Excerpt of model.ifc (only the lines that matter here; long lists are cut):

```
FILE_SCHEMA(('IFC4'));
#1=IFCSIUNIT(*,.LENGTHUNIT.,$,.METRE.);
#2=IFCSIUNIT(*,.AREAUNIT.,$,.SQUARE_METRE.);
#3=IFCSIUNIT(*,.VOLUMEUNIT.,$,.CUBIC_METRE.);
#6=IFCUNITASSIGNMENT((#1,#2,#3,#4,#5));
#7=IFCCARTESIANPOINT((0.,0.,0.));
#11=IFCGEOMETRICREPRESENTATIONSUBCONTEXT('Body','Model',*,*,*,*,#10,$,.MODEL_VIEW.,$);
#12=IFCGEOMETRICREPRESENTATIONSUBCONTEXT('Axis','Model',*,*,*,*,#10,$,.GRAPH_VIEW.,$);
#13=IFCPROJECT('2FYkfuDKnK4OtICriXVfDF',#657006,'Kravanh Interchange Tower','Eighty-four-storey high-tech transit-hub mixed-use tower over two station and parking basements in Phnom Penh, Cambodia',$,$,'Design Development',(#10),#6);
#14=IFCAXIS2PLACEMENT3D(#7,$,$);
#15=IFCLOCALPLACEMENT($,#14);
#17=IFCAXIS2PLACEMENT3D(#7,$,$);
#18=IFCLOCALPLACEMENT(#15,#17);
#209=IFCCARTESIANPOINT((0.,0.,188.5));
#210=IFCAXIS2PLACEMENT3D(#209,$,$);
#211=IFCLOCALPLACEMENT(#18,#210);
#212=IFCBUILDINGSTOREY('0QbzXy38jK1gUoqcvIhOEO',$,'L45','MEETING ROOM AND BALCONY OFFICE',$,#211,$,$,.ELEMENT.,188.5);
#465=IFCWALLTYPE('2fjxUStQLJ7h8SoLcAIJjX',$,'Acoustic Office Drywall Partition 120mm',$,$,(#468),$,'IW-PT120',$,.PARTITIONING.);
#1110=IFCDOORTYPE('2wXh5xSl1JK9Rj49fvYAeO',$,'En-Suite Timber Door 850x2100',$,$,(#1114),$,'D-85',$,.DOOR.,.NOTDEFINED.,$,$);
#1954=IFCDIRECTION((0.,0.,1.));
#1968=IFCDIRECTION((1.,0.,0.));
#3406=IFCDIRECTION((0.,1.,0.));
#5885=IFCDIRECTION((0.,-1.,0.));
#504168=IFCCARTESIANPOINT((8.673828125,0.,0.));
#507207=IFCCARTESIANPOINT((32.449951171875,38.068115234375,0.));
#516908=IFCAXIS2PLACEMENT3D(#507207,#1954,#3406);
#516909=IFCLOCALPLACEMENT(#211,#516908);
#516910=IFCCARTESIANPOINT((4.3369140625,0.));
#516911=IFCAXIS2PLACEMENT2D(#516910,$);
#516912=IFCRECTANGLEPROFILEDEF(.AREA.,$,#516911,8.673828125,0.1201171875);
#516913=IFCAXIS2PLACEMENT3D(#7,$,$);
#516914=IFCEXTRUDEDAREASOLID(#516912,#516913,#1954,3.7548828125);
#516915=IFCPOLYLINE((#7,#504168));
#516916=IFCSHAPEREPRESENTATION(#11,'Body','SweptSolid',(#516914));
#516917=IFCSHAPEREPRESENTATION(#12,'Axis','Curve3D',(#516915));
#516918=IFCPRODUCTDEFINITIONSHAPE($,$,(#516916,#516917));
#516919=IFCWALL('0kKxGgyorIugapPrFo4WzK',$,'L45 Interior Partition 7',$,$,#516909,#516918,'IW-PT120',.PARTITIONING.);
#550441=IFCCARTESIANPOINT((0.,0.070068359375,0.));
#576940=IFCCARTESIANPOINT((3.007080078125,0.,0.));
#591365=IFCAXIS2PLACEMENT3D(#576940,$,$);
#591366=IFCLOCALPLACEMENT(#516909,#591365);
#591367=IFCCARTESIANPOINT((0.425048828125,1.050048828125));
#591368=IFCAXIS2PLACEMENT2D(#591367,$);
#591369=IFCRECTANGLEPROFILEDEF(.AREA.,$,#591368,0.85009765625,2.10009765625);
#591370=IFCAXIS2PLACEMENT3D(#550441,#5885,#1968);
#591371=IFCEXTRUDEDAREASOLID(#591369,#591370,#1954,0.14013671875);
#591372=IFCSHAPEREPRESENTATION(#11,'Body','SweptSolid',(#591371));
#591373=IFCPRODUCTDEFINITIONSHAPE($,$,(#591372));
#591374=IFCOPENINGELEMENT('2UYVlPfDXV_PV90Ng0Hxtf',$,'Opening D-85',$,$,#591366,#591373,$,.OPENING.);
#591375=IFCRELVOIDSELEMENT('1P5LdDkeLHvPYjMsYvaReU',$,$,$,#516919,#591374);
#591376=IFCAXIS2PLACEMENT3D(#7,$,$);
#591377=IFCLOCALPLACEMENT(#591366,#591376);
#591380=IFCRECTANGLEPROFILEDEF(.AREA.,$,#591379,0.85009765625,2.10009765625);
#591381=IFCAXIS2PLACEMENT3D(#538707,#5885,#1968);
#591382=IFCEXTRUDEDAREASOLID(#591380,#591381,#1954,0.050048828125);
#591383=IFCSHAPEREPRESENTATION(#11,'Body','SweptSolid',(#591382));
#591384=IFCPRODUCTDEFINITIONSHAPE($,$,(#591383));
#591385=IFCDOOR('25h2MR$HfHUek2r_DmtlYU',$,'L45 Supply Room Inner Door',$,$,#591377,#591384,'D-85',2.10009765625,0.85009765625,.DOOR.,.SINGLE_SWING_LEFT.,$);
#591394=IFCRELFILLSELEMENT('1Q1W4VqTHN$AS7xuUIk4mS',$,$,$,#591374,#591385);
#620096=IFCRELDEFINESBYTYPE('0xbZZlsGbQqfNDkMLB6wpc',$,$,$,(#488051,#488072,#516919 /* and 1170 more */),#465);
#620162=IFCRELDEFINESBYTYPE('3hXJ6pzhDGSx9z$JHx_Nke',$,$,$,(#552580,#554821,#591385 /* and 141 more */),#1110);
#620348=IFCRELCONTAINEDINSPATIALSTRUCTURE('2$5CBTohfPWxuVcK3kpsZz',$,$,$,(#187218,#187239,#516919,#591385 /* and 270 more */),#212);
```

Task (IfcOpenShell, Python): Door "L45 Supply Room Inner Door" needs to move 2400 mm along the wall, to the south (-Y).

```python
import ifcopenshell
import ifcopenshell.api.geometry
import ifcopenshell.util.placement

model = ifcopenshell.open("model.ifc")

door = model.by_guid("25h2MR$HfHUek2r_DmtlYU")
opening = door.FillsVoids[0].RelatingOpeningElement
wall = opening.VoidsElements[0].RelatingBuildingElement

wall_matrix = ifcopenshell.util.placement.get_local_placement(wall.ObjectPlacement)
shift = wall_matrix[:3, 0] * -2.4
before = ifcopenshell.util.placement.get_local_placement(door.ObjectPlacement)[:3, 3].copy()

# The door is placed relative to its opening, so it follows when the opening moves.
matrix = ifcopenshell.util.placement.get_local_placement(opening.ObjectPlacement)
matrix[:3, 3] += shift
ifcopenshell.api.geometry.edit_object_placement(
    model, product=opening, matrix=matrix, is_si=False, should_transform_children=True
)

after = ifcopenshell.util.placement.get_local_placement(door.ObjectPlacement)[:3, 3]
print("door moved by", (after - before).round(3) + 0.0)

model.write("model_updated.ifc")
```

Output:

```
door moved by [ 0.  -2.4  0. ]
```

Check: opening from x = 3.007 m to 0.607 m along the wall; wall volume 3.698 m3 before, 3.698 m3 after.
